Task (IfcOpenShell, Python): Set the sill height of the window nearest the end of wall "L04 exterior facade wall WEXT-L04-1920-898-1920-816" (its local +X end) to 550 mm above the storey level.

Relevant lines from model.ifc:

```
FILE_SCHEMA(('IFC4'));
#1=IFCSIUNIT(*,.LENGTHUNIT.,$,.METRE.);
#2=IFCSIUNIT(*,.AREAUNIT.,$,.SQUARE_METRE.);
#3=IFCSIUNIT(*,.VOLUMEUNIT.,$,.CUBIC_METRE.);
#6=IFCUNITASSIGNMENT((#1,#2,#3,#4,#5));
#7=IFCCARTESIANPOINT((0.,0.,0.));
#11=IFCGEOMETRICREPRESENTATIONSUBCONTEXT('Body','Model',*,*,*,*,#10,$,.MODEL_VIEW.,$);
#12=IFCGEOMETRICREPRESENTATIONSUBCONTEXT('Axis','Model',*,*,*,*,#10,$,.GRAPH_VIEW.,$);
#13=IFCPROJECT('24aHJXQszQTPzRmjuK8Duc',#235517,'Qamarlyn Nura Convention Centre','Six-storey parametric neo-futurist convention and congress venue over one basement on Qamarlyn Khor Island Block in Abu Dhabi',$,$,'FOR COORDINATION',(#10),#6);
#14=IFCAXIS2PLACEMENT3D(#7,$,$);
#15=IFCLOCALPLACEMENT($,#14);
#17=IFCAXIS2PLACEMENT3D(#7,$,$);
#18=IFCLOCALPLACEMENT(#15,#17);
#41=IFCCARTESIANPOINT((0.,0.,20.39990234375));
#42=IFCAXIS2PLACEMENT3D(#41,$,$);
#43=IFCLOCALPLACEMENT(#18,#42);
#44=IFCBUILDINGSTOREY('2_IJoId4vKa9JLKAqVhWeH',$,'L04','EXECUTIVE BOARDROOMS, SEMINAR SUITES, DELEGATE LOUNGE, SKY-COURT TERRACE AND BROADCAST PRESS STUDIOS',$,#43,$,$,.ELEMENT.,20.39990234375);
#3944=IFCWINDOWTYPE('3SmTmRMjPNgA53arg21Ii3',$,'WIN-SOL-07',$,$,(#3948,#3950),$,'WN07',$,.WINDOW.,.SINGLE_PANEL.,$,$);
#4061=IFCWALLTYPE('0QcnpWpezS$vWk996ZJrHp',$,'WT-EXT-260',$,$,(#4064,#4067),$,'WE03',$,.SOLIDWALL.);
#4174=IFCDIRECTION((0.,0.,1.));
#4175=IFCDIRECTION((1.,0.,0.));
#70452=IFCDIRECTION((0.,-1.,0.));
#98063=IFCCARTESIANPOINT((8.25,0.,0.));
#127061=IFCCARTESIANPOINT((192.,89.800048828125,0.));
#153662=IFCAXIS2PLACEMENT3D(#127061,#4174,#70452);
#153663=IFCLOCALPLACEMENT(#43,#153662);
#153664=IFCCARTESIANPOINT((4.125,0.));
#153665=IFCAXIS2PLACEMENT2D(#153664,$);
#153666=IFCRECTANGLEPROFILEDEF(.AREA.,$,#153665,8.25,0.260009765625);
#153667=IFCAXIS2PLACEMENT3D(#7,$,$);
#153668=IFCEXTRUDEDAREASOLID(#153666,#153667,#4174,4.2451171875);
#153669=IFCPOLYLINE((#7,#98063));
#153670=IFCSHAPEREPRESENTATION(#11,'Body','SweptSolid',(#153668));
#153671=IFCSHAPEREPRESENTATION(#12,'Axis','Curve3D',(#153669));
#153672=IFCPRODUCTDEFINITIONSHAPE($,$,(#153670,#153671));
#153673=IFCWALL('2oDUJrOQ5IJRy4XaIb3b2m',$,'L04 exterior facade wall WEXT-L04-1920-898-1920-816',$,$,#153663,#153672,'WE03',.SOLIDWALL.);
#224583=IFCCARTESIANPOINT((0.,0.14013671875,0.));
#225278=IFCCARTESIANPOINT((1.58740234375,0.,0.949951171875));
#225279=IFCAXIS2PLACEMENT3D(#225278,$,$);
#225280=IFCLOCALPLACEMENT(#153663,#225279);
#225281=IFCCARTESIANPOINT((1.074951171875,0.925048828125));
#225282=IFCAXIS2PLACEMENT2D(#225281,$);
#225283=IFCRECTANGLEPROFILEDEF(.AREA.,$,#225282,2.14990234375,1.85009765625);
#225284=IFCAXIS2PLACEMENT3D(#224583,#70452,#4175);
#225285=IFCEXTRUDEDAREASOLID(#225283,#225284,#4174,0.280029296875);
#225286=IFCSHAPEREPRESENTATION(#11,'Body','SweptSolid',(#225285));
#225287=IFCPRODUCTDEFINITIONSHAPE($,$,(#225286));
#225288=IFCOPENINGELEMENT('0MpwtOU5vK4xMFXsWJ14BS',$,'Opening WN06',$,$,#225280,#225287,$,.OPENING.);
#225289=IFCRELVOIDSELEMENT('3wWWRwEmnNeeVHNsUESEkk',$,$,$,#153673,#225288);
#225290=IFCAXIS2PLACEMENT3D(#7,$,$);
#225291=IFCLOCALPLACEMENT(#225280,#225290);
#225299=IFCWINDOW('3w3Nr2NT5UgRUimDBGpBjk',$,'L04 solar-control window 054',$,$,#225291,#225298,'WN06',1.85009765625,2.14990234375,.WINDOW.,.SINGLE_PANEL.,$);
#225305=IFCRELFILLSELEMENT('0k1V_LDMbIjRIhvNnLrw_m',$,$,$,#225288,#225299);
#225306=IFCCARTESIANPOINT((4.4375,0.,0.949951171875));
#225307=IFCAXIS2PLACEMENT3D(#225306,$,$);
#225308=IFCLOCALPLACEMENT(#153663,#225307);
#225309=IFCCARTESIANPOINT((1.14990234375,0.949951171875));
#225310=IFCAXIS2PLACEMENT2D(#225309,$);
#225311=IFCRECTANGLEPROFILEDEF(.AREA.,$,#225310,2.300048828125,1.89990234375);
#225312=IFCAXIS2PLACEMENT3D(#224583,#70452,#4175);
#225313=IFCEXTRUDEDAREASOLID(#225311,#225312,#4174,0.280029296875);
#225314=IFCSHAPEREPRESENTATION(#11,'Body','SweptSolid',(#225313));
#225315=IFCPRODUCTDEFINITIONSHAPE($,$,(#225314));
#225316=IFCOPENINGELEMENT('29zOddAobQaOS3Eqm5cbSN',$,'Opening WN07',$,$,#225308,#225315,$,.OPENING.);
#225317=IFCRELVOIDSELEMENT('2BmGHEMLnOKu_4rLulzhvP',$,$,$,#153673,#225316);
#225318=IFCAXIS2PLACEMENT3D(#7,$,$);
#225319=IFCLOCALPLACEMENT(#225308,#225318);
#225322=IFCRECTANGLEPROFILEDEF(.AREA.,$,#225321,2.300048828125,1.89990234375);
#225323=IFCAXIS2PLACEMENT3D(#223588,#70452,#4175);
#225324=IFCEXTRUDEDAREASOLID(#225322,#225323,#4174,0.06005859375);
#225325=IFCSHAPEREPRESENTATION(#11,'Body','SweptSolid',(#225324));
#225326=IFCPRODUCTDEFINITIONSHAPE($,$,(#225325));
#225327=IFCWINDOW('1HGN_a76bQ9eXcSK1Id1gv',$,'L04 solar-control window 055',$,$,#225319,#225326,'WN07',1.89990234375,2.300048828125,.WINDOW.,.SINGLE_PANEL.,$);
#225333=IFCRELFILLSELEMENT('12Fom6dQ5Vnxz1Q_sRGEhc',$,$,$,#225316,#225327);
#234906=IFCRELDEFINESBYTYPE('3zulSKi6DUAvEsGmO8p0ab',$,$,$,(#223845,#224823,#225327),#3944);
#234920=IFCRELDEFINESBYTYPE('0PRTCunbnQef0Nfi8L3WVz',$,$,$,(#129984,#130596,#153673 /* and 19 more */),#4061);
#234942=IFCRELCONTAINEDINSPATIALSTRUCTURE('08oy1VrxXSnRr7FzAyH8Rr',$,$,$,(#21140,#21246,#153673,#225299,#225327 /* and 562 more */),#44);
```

```python
import numpy as np
import ifcopenshell
import ifcopenshell.api.geometry
import ifcopenshell.geom
import ifcopenshell.util.element
import ifcopenshell.util.placement
import ifcopenshell.util.shape
import ifcopenshell.util.unit

model = ifcopenshell.open("model.ifc")
unit_scale = ifcopenshell.util.unit.calculate_unit_scale(model)

window = model.by_guid("1HGN_a76bQ9eXcSK1Id1gv")
opening = window.FillsVoids[0].RelatingOpeningElement
storey = ifcopenshell.util.element.get_container(window, ifc_class="IfcBuildingStorey")
level = ifcopenshell.util.placement.get_local_placement(storey.ObjectPlacement)[2, 3]

# The opening's origin need not be at the sill, so measure its lowest point.
shape = ifcopenshell.geom.create_shape(ifcopenshell.geom.settings(), opening)
bottom = ifcopenshell.util.shape.get_shape_bottom_elevation(shape, shape.geometry) / unit_scale
dz = level + 0.55 / unit_scale - bottom

shift = np.array([0.0, 0.0, dz])
# The window is placed relative to its opening, so it follows when the opening moves.
matrix = ifcopenshell.util.placement.get_local_placement(opening.ObjectPlacement)
matrix[:3, 3] += shift
ifcopenshell.api.geometry.edit_object_placement(
    model, product=opening, matrix=matrix, is_si=False, should_transform_children=True
)

print(f"moved by {dz * unit_scale:+.3f} m")

model.write("model_edited.ifc")
```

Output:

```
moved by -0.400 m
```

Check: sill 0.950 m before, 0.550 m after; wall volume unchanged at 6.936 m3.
